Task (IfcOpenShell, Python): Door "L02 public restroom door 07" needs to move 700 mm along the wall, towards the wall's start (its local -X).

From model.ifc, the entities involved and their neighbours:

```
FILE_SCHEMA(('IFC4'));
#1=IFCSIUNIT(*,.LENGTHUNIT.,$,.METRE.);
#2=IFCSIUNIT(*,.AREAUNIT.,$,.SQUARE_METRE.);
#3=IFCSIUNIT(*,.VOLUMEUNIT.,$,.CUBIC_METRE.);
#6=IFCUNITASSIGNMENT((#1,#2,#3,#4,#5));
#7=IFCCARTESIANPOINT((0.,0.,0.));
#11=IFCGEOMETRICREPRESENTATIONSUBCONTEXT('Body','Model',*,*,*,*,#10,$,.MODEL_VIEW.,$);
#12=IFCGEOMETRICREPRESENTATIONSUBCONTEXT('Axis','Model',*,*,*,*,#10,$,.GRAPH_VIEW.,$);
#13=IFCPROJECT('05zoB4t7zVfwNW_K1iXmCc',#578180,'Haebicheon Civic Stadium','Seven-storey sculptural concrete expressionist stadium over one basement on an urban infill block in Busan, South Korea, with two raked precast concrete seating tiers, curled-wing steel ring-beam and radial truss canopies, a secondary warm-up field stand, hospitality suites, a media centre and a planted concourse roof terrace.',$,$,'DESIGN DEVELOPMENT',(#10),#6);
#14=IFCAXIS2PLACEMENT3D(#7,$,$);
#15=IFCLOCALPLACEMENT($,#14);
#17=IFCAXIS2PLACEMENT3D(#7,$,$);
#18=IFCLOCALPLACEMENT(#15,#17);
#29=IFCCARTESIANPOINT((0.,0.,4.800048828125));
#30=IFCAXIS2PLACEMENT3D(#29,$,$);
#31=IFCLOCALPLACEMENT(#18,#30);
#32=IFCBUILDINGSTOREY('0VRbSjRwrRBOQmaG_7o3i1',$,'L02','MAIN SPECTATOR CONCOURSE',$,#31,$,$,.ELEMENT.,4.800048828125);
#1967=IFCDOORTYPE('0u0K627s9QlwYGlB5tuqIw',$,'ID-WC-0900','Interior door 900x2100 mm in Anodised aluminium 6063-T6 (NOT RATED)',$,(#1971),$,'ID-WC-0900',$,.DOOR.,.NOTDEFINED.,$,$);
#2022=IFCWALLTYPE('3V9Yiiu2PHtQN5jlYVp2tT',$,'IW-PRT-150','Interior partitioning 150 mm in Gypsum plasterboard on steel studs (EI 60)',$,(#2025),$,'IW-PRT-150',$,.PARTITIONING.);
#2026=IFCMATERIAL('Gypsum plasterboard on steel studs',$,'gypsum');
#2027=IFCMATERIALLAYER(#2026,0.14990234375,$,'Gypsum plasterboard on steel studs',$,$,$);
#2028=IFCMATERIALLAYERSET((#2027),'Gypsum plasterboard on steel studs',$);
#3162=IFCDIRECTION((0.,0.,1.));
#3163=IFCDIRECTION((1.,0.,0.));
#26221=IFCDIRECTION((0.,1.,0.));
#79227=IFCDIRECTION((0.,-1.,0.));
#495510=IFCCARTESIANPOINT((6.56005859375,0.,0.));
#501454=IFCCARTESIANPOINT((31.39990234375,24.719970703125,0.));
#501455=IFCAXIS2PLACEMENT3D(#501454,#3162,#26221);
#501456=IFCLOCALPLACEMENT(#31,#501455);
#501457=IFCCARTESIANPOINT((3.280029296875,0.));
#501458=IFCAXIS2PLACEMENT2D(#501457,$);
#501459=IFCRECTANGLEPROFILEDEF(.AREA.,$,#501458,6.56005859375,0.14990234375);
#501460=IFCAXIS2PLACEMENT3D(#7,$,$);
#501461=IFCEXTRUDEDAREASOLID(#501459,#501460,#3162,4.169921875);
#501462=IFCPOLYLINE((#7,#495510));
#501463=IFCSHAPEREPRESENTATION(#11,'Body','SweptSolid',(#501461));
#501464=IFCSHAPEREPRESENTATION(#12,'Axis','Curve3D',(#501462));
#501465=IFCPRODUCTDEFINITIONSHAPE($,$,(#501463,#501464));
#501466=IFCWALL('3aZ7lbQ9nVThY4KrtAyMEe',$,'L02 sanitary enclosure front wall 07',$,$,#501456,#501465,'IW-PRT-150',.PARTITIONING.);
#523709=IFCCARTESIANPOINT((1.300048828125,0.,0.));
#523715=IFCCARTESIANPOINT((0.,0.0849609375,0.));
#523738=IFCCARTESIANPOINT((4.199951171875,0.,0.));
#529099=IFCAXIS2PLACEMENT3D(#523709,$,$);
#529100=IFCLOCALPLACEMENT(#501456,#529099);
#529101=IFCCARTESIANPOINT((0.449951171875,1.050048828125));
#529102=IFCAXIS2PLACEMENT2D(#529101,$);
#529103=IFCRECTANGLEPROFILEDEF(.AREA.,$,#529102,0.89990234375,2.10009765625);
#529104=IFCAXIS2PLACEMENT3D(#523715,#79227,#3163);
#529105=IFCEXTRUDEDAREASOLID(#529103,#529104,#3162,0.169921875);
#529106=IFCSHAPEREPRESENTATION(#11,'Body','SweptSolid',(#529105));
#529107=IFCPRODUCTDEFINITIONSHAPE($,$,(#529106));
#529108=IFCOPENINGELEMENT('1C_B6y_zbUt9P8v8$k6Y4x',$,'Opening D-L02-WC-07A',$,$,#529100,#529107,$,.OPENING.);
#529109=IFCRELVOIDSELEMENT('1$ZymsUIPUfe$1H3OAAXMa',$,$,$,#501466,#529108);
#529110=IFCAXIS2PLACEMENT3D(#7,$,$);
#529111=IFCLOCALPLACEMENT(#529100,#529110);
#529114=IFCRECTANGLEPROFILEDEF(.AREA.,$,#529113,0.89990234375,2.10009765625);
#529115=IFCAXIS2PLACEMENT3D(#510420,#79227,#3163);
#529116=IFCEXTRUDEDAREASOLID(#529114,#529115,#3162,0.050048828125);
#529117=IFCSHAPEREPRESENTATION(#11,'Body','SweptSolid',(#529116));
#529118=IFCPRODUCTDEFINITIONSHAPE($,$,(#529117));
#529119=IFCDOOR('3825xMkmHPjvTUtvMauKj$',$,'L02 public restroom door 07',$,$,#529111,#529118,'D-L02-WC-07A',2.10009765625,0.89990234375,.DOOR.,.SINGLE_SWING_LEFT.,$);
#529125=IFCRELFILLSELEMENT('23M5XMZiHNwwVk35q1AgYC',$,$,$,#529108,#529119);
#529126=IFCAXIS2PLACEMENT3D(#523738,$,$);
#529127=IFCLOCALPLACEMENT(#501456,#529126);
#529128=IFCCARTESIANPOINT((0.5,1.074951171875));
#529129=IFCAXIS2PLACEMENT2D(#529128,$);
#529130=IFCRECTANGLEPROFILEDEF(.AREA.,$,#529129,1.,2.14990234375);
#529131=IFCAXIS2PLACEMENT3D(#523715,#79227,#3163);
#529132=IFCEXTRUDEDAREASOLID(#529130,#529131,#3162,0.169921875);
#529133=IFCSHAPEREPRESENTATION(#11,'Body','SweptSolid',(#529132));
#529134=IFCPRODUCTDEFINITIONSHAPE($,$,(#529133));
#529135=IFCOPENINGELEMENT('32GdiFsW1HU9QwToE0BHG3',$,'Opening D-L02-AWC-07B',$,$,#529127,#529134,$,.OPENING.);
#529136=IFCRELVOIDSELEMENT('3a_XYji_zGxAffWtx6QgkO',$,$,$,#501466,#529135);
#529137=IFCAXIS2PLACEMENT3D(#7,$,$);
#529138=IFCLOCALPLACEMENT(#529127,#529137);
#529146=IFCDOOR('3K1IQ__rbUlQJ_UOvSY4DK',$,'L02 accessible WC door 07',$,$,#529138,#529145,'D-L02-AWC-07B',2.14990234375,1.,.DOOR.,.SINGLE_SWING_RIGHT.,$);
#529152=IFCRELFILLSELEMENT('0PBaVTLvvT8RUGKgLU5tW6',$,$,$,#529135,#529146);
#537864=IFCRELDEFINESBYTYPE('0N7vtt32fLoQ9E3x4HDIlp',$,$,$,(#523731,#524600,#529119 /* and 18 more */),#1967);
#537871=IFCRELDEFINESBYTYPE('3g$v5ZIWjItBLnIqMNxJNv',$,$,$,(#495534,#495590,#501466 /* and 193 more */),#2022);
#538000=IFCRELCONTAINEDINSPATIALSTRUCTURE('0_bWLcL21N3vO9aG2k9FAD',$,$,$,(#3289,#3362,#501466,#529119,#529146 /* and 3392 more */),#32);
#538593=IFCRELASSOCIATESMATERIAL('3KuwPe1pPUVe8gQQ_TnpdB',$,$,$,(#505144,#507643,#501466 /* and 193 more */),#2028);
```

```python
import ifcopenshell
import ifcopenshell.api.geometry
import ifcopenshell.util.placement
import ifcopenshell.util.unit

model = ifcopenshell.open("model.ifc")
unit_scale = ifcopenshell.util.unit.calculate_unit_scale(model)

door = model.by_id(529119)
opening = door.FillsVoids[0].RelatingOpeningElement
wall = opening.VoidsElements[0].RelatingBuildingElement

wall_matrix = ifcopenshell.util.placement.get_local_placement(wall.ObjectPlacement)
shift = wall_matrix[:3, 0] * -0.7 / unit_scale
before = ifcopenshell.util.placement.get_local_placement(door.ObjectPlacement)[:3, 3].copy()

# The door is placed relative to its opening, so it follows when the opening moves.
matrix = ifcopenshell.util.placement.get_local_placement(opening.ObjectPlacement)
matrix[:3, 3] += shift
ifcopenshell.api.geometry.edit_object_placement(
    model, product=opening, matrix=matrix, is_si=False, should_transform_children=True
)

after = ifcopenshell.util.placement.get_local_placement(door.ObjectPlacement)[:3, 3]
print("door moved by", (after - before).round(3) + 0.0)

model.write("model_updated.ifc")
```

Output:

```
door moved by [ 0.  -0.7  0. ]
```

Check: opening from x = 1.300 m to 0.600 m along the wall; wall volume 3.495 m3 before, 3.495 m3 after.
